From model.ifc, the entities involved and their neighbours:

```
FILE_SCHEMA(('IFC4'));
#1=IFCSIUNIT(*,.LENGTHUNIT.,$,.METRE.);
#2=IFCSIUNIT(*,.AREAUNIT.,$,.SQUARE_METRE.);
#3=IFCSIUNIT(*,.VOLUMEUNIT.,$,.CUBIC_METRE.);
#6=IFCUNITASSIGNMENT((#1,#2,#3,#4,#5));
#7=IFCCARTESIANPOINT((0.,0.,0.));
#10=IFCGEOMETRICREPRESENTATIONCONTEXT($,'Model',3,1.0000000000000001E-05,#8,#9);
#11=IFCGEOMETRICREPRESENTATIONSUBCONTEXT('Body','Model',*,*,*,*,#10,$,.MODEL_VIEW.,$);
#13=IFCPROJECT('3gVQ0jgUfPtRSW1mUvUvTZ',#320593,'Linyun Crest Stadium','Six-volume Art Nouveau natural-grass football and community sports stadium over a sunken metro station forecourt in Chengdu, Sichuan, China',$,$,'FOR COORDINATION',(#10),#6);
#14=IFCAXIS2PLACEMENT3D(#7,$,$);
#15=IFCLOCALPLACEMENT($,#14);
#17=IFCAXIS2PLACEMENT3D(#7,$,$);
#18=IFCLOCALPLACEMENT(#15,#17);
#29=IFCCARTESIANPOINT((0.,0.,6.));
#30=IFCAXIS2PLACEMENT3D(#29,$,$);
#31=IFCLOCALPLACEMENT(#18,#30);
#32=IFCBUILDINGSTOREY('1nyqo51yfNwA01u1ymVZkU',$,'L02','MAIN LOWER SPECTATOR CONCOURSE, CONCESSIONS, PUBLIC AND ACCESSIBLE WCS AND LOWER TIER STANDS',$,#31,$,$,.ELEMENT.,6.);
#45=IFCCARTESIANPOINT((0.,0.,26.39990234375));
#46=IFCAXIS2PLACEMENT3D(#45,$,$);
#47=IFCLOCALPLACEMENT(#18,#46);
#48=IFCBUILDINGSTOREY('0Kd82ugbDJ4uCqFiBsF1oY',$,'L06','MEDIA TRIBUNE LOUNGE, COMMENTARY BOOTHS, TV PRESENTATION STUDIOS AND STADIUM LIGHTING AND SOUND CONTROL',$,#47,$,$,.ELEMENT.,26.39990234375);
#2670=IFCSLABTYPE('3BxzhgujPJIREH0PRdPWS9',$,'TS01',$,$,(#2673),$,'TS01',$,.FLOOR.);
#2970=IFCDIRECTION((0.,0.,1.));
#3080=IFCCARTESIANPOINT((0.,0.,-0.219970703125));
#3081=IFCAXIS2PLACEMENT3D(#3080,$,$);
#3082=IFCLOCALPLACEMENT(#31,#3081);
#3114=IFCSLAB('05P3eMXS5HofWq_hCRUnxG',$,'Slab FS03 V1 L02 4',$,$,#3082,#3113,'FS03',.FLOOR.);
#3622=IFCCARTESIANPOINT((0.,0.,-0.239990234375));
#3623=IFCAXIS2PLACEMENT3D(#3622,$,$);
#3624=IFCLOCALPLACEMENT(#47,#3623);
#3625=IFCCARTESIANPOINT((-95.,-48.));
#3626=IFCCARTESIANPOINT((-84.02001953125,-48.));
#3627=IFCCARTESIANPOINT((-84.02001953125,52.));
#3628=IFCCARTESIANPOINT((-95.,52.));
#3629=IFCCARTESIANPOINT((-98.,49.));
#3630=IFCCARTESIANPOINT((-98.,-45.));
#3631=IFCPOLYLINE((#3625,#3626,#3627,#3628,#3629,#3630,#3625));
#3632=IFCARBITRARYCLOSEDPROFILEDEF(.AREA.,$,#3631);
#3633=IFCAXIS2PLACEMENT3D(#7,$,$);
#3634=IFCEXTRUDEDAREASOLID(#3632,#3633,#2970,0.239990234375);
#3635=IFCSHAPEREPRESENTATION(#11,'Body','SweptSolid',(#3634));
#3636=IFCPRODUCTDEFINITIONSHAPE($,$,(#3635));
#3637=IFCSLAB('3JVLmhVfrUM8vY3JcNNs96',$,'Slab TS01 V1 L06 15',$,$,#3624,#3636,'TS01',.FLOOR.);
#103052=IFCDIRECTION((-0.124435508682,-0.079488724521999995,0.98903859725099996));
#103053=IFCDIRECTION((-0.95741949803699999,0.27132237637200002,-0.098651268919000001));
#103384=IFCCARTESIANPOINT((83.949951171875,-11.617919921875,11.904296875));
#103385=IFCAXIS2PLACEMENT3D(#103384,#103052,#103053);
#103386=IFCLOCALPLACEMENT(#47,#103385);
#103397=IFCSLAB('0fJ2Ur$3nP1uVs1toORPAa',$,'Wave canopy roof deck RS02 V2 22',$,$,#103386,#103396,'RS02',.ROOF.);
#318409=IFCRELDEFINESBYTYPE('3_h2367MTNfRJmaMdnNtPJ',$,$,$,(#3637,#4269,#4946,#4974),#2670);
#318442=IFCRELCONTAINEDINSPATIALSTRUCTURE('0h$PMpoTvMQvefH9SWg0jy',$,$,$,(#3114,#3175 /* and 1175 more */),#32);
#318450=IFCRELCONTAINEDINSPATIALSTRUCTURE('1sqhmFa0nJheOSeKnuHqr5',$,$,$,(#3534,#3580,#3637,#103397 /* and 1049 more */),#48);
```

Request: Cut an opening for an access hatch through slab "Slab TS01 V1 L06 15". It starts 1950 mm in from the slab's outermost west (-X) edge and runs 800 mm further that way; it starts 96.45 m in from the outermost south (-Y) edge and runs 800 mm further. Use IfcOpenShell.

```python
import numpy as np
import ifcopenshell
import ifcopenshell.api.feature
import ifcopenshell.api.geometry
import ifcopenshell.api.root
import ifcopenshell.geom
import ifcopenshell.util.placement
import ifcopenshell.util.representation
import ifcopenshell.util.shape
import ifcopenshell.util.unit

model = ifcopenshell.open("model.ifc")
unit_scale = ifcopenshell.util.unit.calculate_unit_scale(model)
settings = ifcopenshell.geom.settings()


def volume(element):
    """Net volume in cubic metres, openings subtracted."""
    shape = ifcopenshell.geom.create_shape(settings, element)
    return ifcopenshell.util.shape.get_volume(shape.geometry)


slab = model.by_guid("3JVLmhVfrUM8vY3JcNNs96")
before = volume(slab)

# Extent in the slab's own axes, in metres. The edges named are its -X and -Y sides.
slab_shape = ifcopenshell.geom.create_shape(settings, slab)
vertices = ifcopenshell.util.shape.get_vertices(slab_shape.geometry)
x_min, y_min, bottom = vertices.min(axis=0)
top = vertices[:, 2].max()

opening = ifcopenshell.api.root.create_entity(model, ifc_class="IfcOpeningElement", name="Access hatch opening", predefined_type="OPENING")
context = ifcopenshell.util.representation.get_context(model, "Model", "Body", "MODEL_VIEW")
width, depth = 0.8, 0.8
outline = [(0.0, 0.0), (width, 0.0), (width, depth), (0.0, depth), (0.0, 0.0)]
# Overshoot both faces by 50 mm so the cut is clean.
shape = ifcopenshell.api.geometry.add_slab_representation(
    model, context=context, depth=top - bottom + 0.1, polyline=outline
)
ifcopenshell.api.geometry.assign_representation(model, product=opening, representation=shape)

matrix = ifcopenshell.util.placement.get_local_placement(slab.ObjectPlacement)
matrix[:, 3] = matrix @ np.append(np.array([x_min + 1.95, y_min + 96.45, bottom - 0.05]) / unit_scale, 1.0)
ifcopenshell.api.geometry.edit_object_placement(model, product=opening, matrix=matrix, is_si=False)
ifcopenshell.api.feature.add_feature(model, feature=opening, element=slab)

after = volume(slab)

print(f"slab volume {before:.3f} -> {after:.3f} m3")

model.write("model-out.ifc")
```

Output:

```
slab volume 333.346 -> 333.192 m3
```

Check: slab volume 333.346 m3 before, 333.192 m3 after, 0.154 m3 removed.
